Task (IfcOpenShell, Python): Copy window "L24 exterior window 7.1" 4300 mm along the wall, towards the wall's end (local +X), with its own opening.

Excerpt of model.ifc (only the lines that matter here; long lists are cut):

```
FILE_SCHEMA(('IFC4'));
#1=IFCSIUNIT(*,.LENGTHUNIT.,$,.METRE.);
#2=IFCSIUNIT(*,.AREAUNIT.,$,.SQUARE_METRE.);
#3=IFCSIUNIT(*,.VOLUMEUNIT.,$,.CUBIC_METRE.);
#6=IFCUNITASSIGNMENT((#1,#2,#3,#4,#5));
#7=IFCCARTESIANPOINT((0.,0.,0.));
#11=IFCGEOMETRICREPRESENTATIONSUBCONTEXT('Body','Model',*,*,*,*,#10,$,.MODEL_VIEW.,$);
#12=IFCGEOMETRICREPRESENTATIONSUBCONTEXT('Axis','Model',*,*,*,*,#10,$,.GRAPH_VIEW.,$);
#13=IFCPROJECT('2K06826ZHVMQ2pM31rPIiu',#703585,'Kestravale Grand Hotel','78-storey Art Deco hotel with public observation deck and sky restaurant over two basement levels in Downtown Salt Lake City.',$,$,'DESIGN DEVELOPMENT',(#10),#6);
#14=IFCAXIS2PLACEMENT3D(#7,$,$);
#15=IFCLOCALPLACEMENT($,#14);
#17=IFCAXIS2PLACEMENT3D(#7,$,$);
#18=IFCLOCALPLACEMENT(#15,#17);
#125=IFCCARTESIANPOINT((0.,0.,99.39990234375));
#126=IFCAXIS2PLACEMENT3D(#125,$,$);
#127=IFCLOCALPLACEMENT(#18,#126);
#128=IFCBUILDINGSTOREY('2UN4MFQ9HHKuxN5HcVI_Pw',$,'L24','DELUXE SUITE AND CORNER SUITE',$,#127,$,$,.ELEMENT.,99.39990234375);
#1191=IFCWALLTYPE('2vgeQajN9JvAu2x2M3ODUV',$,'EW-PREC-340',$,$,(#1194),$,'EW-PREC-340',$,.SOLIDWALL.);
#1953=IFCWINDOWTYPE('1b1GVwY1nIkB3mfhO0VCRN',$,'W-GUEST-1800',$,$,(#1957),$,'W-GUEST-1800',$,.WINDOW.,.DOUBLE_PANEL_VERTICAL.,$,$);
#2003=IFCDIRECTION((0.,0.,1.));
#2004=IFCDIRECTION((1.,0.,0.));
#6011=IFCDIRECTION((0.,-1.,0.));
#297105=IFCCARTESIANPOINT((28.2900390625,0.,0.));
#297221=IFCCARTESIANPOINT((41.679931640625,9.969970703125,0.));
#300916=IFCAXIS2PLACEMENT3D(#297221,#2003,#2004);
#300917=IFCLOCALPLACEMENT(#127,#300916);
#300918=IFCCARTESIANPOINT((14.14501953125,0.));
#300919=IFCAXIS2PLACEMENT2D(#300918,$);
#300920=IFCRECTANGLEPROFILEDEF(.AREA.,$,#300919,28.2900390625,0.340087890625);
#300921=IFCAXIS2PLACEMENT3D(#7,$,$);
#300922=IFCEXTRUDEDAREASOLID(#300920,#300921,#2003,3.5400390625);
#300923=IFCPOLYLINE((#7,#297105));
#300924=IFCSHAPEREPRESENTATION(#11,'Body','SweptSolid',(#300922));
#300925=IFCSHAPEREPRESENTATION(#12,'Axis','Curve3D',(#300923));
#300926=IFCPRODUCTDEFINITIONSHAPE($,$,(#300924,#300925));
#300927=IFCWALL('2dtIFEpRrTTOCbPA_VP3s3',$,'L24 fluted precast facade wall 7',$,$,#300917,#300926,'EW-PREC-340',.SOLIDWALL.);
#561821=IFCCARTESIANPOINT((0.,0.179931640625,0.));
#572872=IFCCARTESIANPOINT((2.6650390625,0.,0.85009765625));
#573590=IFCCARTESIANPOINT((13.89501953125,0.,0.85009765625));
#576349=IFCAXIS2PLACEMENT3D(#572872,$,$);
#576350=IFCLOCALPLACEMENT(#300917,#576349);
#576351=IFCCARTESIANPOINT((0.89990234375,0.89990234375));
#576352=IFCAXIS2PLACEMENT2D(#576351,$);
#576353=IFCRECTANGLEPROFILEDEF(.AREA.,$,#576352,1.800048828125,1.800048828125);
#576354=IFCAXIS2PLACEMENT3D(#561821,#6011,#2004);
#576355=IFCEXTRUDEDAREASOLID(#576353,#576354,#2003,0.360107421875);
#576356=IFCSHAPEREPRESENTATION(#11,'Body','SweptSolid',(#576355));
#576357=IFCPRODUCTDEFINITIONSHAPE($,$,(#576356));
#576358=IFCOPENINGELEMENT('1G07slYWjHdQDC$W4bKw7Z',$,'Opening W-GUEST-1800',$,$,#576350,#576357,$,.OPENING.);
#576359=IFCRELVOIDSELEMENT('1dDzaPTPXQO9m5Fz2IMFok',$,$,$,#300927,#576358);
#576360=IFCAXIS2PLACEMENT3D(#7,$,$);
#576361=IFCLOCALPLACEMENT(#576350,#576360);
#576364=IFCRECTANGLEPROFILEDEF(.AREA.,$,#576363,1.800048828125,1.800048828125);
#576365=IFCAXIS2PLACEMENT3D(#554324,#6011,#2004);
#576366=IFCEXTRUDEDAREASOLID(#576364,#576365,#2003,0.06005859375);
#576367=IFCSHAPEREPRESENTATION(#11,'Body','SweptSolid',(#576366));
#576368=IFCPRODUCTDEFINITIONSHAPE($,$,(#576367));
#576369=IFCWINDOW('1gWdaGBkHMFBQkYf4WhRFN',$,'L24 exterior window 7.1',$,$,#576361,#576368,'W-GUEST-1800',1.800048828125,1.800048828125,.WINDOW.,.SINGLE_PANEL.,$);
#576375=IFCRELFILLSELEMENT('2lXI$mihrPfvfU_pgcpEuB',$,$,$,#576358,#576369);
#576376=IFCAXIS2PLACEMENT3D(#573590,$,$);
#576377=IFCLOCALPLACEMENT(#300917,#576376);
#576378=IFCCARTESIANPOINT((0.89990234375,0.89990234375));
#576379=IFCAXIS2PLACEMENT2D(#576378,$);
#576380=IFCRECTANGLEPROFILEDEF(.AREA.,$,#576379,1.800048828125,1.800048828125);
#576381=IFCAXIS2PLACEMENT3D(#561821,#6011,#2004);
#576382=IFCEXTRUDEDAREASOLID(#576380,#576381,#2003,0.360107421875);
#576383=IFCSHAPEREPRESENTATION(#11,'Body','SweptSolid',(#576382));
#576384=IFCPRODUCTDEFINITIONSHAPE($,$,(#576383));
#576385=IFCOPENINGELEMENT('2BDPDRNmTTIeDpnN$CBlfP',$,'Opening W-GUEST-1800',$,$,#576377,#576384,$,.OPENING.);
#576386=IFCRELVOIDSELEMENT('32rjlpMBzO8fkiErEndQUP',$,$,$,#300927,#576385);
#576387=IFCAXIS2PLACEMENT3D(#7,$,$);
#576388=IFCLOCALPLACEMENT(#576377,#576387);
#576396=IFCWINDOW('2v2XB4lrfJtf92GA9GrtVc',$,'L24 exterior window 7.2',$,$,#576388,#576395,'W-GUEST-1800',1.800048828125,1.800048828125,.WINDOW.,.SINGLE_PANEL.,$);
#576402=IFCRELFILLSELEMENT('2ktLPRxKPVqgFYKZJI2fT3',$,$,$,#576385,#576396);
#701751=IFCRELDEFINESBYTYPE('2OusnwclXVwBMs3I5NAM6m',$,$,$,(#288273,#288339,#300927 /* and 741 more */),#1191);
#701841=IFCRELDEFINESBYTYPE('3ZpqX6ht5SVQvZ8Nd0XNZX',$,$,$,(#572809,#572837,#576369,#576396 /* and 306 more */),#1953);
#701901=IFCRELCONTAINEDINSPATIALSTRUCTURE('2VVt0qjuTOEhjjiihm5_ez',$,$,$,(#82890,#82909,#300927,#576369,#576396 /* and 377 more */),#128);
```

```python
import ifcopenshell
import ifcopenshell.api.feature
import ifcopenshell.api.geometry
import ifcopenshell.api.root
import ifcopenshell.geom
import ifcopenshell.util.element
import ifcopenshell.util.placement
import ifcopenshell.util.shape

model = ifcopenshell.open("model.ifc")
settings = ifcopenshell.geom.settings()


def volume(element):
    """Net volume in cubic metres, openings subtracted."""
    shape = ifcopenshell.geom.create_shape(settings, element)
    return ifcopenshell.util.shape.get_volume(shape.geometry)


window = model.by_guid("1gWdaGBkHMFBQkYf4WhRFN")
opening = window.FillsVoids[0].RelatingOpeningElement
wall = opening.VoidsElements[0].RelatingBuildingElement
before = volume(wall)
shift = ifcopenshell.util.placement.get_local_placement(wall.ObjectPlacement)[:3, 0] * 4.3

# copy_class copies the void relationship, type, container and properties, but no geometry.
new_opening = ifcopenshell.api.root.copy_class(model, product=opening)
new_opening.Representation = ifcopenshell.util.element.copy_deep(
    model, opening.Representation, exclude=["IfcGeometricRepresentationContext", "IfcRepresentationMap"]
)
new_window = ifcopenshell.api.root.copy_class(model, product=window)
new_window.Representation = ifcopenshell.util.element.copy_deep(
    model, window.Representation, exclude=["IfcGeometricRepresentationContext", "IfcRepresentationMap"]
)
new_window.Tag = None
ifcopenshell.api.feature.add_filling(model, opening=new_opening, element=new_window)

for old, new in ((opening, new_opening), (window, new_window)):
    matrix = ifcopenshell.util.placement.get_local_placement(old.ObjectPlacement)
    matrix[:3, 3] += shift
    ifcopenshell.api.geometry.edit_object_placement(model, product=new, matrix=matrix, is_si=False)

after = volume(wall)

print(f"wall volume {before:.3f} -> {after:.3f} m3")

model.write("model_updated.ifc")
```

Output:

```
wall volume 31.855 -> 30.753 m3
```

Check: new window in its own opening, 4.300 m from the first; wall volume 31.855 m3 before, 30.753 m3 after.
